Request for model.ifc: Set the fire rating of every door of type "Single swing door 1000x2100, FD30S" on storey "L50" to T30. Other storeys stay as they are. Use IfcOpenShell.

First a look at what the model holds.

```python
import ifcopenshell
import ifcopenshell.util.element

model = ifcopenshell.open("model.ifc")
print(model.schema)
storey = next(s for s in model.by_type("IfcBuildingStorey") if s.Name == "L50")
doors = [e for e in ifcopenshell.util.element.get_decomposition(storey) if e.is_a("IfcDoor")]
seen = {}
for e in doors:
    element_type = ifcopenshell.util.element.get_type(e)
    key = (element_type.Name if element_type != e and element_type else None, ifcopenshell.util.element.get_pset(e, "Pset_DoorCommon", "FireRating"))
    seen[key] = seen.get(key, 0) + 1
for (name, value), count in sorted(seen.items(), key=str):
    print(count, "x", name, "|", value)
```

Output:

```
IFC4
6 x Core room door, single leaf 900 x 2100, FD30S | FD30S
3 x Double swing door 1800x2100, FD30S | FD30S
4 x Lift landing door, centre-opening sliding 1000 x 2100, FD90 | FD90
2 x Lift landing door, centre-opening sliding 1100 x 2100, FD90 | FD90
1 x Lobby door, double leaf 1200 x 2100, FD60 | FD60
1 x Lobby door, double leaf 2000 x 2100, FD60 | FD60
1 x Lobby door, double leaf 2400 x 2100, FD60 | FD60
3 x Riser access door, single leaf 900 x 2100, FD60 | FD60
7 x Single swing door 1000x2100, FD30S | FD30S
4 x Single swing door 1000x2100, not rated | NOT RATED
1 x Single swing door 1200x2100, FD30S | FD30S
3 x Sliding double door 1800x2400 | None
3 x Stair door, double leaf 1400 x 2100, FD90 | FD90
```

```python
import ifcopenshell
import ifcopenshell.api.pset
import ifcopenshell.util.element

model = ifcopenshell.open("model.ifc")

storey = next(s for s in model.by_type("IfcBuildingStorey") if s.Name == "L50")
doors = [e for e in ifcopenshell.util.element.get_decomposition(storey) if e.is_a("IfcDoor")]

count = 0
for e in doors:
    element_type = ifcopenshell.util.element.get_type(e)
    if element_type in (None, e) or element_type.Name != "Single swing door 1000x2100, FD30S":
        continue
    # add_pset returns the element's existing set when there is one.
    pset = ifcopenshell.api.pset.add_pset(model, product=e, name="Pset_DoorCommon")
    ifcopenshell.api.pset.edit_pset(model, pset=pset, properties={"FireRating": "T30"})
    count += 1

print(count, "doors updated")

model.write("model-out.ifc")
```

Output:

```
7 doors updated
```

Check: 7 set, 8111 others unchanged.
